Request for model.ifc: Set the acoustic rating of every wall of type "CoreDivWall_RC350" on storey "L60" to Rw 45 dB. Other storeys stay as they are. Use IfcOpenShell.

First a look at what the model holds.

```python
import ifcopenshell
import ifcopenshell.util.element

model = ifcopenshell.open("model.ifc")
print(model.schema)
storey = next(s for s in model.by_type("IfcBuildingStorey") if s.Name == "L60")
walls = [e for e in ifcopenshell.util.element.get_decomposition(storey) if e.is_a("IfcWall")]
seen = {}
for e in walls:
    element_type = ifcopenshell.util.element.get_type(e)
    key = (element_type.Name if element_type != e and element_type else None, ifcopenshell.util.element.get_pset(e, "Pset_WallCommon", "AcousticRating"))
    seen[key] = seen.get(key, 0) + 1
for (name, value), count in sorted(seen.items(), key=str):
    print(count, "x", name, "|", value)
```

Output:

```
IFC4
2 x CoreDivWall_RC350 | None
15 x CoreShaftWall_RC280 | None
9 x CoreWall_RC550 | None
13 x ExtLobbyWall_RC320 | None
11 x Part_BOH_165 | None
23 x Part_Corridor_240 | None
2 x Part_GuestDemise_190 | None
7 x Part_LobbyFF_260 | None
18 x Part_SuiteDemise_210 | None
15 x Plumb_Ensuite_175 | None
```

```python
import ifcopenshell
import ifcopenshell.api.pset
import ifcopenshell.util.element

model = ifcopenshell.open("model.ifc")

storey = next(s for s in model.by_type("IfcBuildingStorey") if s.Name == "L60")
walls = [e for e in ifcopenshell.util.element.get_decomposition(storey) if e.is_a("IfcWall")]

count = 0
for e in walls:
    element_type = ifcopenshell.util.element.get_type(e)
    if element_type in (None, e) or element_type.Name != "CoreDivWall_RC350":
        continue
    found = ifcopenshell.util.element.get_pset(e, "Pset_WallCommon", should_inherit=False)
    if found:
        pset = model.by_id(found["id"])
        if len(ifcopenshell.util.element.get_elements_by_pset(pset)) > 1:
            pset = ifcopenshell.api.pset.unshare_pset(model, products=[e], pset=pset)[0]
    else:
        pset = ifcopenshell.api.pset.add_pset(model, product=e, name="Pset_WallCommon")
    ifcopenshell.api.pset.edit_pset(model, pset=pset, properties={"AcousticRating": "Rw 45 dB"})
    count += 1

print(count, "walls updated")

model.write("model_rev.ifc")
```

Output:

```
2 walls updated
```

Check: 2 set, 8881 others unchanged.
